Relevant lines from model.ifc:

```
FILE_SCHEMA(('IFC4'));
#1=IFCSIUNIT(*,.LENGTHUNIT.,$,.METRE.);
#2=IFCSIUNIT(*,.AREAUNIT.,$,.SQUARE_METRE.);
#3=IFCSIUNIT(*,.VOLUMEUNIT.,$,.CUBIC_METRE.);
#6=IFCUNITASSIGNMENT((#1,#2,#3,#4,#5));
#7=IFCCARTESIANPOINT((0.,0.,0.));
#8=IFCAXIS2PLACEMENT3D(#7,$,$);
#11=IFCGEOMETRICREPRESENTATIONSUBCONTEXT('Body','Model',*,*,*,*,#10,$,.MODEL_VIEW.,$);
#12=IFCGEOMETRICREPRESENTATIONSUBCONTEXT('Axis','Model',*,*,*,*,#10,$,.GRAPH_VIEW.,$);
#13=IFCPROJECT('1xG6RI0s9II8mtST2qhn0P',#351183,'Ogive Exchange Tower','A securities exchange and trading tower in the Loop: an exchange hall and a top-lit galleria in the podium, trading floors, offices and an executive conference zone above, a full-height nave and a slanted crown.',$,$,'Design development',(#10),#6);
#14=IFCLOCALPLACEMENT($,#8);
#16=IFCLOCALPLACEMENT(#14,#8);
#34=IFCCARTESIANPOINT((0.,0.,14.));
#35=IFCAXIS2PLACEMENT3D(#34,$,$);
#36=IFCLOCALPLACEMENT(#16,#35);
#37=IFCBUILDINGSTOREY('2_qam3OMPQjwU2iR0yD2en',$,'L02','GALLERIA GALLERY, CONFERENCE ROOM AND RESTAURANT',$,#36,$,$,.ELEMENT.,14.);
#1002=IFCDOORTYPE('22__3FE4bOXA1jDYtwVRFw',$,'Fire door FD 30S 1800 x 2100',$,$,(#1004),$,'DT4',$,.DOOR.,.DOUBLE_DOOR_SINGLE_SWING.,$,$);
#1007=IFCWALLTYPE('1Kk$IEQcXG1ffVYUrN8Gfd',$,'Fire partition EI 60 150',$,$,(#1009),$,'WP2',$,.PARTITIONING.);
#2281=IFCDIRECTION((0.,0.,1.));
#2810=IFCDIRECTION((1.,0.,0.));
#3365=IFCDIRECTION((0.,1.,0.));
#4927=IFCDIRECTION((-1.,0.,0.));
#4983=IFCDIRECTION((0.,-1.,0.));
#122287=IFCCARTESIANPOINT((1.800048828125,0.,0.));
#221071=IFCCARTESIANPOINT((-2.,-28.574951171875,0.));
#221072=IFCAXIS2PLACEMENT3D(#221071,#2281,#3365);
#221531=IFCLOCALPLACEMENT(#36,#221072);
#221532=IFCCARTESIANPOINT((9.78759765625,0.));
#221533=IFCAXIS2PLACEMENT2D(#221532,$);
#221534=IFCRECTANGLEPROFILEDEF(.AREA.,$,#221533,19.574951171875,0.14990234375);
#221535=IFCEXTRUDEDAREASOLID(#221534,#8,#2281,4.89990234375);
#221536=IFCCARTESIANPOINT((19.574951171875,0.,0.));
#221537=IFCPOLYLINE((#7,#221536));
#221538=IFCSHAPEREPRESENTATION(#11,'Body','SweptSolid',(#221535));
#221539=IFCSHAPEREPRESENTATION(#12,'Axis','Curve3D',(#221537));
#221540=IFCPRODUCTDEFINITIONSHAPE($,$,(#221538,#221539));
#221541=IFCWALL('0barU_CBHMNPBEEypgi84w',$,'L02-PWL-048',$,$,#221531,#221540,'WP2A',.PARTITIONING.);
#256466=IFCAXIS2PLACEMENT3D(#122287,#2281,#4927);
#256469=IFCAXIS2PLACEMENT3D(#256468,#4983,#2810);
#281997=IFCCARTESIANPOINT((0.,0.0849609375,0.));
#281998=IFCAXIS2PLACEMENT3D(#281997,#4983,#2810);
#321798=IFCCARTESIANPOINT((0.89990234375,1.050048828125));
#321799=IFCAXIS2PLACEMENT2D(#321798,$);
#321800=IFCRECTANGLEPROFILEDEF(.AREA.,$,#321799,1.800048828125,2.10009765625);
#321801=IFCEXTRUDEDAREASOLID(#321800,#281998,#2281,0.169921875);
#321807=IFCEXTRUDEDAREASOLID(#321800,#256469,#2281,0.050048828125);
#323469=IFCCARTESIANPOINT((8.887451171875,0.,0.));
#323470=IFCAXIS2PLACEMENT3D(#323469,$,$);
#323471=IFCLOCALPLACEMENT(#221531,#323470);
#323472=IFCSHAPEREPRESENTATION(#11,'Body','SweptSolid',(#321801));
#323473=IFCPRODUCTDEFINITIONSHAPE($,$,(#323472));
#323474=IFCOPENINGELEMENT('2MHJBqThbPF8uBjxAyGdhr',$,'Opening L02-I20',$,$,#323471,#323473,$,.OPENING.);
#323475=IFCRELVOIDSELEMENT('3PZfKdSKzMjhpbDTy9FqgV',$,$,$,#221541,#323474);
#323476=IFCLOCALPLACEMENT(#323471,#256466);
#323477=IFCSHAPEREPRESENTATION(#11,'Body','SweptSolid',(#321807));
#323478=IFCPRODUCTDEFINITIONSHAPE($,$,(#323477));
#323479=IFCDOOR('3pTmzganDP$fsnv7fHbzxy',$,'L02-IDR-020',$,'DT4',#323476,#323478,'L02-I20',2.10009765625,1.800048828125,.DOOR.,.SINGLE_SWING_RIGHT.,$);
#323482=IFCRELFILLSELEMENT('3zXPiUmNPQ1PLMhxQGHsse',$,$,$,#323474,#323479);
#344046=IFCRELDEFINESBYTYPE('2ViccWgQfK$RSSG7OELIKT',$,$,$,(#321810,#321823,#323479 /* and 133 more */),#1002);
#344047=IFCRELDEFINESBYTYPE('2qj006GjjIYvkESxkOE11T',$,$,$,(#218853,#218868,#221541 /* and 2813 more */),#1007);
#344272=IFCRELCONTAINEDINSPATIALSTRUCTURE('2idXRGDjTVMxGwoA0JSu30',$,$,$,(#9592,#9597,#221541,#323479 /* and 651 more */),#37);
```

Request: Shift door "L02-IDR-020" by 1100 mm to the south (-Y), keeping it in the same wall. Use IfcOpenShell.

```python
import ifcopenshell
import ifcopenshell.api.geometry
import ifcopenshell.util.placement

model = ifcopenshell.open("model.ifc")

door = model.by_guid("3pTmzganDP$fsnv7fHbzxy")
opening = door.FillsVoids[0].RelatingOpeningElement
wall = opening.VoidsElements[0].RelatingBuildingElement

wall_matrix = ifcopenshell.util.placement.get_local_placement(wall.ObjectPlacement)
shift = wall_matrix[:3, 0] * -1.1
before = ifcopenshell.util.placement.get_local_placement(door.ObjectPlacement)[:3, 3].copy()

# The door is placed relative to its opening, so it follows when the opening moves.
matrix = ifcopenshell.util.placement.get_local_placement(opening.ObjectPlacement)
matrix[:3, 3] += shift
ifcopenshell.api.geometry.edit_object_placement(
    model, product=opening, matrix=matrix, is_si=False, should_transform_children=True
)

after = ifcopenshell.util.placement.get_local_placement(door.ObjectPlacement)[:3, 3]
print("door moved by", (after - before).round(3) + 0.0)

model.write("model-out.ifc")
```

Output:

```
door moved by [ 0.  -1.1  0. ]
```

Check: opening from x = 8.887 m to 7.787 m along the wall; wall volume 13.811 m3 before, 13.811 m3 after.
